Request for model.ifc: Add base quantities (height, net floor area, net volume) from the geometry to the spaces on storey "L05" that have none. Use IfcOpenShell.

First a look at what the model holds.

```python
import ifcopenshell
import ifcopenshell.util.element
import ifcopenshell.util.unit

model = ifcopenshell.open("model.ifc")
print(model.schema)
for unit_type in ("LENGTHUNIT", "AREAUNIT", "VOLUMEUNIT"):
    print(unit_type, ifcopenshell.util.unit.calculate_unit_scale(model, unit_type))
storey = next(s for s in model.by_type("IfcBuildingStorey") if s.Name == "L05")
spaces = [e for e in ifcopenshell.util.element.get_decomposition(storey) if e.is_a("IfcSpace")]
for e in sorted(spaces, key=lambda e: e.id()):
    print(e.id(), e.is_a(), e.Name, list(ifcopenshell.util.element.get_psets(e, qtos_only=True)), sep=" | ")
```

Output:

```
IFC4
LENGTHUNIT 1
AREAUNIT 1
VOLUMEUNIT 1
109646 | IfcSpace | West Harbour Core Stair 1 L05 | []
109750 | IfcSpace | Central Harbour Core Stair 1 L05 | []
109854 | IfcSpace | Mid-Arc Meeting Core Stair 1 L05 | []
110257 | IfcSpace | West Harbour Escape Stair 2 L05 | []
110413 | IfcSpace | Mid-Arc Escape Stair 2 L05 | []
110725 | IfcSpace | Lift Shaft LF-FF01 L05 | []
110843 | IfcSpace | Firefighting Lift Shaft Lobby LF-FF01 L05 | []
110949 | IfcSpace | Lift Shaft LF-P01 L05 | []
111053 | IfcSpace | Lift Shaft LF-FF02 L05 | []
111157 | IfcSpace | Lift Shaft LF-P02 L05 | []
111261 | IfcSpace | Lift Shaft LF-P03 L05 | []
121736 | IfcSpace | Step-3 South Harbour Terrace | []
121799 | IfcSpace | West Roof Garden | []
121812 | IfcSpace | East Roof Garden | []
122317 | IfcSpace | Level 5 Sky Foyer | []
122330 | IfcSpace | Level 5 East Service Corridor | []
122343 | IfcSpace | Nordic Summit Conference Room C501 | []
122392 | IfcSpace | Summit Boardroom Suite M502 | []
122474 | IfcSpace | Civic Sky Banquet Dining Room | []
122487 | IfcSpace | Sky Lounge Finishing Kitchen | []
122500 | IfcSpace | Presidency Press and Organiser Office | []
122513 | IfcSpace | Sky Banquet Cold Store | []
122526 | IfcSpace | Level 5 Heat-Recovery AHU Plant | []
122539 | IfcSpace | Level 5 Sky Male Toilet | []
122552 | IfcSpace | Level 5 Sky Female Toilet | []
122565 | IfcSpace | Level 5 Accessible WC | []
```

```python
import ifcopenshell
import ifcopenshell.api.pset
import ifcopenshell.geom
import ifcopenshell.util.element
import ifcopenshell.util.shape
import ifcopenshell.util.unit

model = ifcopenshell.open("model.ifc")
unit_scale = ifcopenshell.util.unit.calculate_unit_scale(model)
area_scale = ifcopenshell.util.unit.calculate_unit_scale(model, "AREAUNIT")
volume_scale = ifcopenshell.util.unit.calculate_unit_scale(model, "VOLUMEUNIT")
settings = ifcopenshell.geom.settings()

storey = next(s for s in model.by_type("IfcBuildingStorey") if s.Name == "L05")
spaces = [e for e in ifcopenshell.util.element.get_decomposition(storey) if e.is_a("IfcSpace")]

for e in sorted(spaces, key=lambda e: e.id()):
    if ifcopenshell.util.element.get_psets(e, qtos_only=True, should_inherit=False):
        continue
    # Geometry comes back in metres, in the element's own axes.
    shape = ifcopenshell.geom.create_shape(settings, e)
    values = {
        "Height": ifcopenshell.util.shape.get_z(shape.geometry) / unit_scale,
        "NetFloorArea": ifcopenshell.util.shape.get_footprint_area(shape.geometry) / area_scale,
        "NetVolume": ifcopenshell.util.shape.get_volume(shape.geometry) / volume_scale,
    }
    qto = ifcopenshell.api.pset.add_qto(model, product=e, name="Qto_SpaceBaseQuantities")
    ifcopenshell.api.pset.edit_qto(model, qto=qto, properties=values)
    print(e.id(), {k: round(v, 3) for k, v in values.items()})

model.write("model_updated.ifc")
```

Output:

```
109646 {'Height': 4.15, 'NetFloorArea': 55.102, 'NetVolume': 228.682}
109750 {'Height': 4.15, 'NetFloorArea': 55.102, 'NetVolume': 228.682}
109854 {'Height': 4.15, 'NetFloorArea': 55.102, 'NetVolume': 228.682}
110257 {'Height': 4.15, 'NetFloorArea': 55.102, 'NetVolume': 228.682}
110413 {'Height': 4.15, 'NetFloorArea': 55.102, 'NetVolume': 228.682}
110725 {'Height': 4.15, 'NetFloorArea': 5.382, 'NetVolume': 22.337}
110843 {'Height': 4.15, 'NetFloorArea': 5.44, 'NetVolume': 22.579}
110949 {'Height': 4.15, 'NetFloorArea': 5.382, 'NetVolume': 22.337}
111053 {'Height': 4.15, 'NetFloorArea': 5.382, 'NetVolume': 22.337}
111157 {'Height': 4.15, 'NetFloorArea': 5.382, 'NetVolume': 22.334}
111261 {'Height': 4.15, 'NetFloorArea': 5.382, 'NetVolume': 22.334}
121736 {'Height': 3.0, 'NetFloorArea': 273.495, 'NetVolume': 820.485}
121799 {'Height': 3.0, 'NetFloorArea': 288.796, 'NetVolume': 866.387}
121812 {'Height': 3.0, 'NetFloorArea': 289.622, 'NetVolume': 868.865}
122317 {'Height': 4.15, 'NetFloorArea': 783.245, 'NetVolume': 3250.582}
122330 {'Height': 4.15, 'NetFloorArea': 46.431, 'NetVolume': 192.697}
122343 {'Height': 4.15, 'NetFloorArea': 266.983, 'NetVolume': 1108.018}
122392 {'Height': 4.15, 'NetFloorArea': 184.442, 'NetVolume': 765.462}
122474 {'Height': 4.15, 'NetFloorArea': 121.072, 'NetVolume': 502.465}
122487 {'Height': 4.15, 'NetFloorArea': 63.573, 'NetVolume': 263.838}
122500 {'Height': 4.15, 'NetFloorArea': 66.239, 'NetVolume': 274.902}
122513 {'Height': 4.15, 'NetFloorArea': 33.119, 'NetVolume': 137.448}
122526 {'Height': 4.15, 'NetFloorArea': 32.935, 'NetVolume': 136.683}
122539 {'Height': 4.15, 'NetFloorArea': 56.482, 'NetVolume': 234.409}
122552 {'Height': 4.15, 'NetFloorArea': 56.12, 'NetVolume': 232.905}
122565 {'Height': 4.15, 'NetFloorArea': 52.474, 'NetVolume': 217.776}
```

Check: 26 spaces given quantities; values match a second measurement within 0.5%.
